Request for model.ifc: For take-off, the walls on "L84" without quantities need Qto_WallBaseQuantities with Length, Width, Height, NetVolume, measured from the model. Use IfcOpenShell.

First a look at what the model holds.

```python
import ifcopenshell
import ifcopenshell.util.element
import ifcopenshell.util.unit

model = ifcopenshell.open("model.ifc")
print(model.schema)
for unit_type in ("LENGTHUNIT", "AREAUNIT", "VOLUMEUNIT"):
    print(unit_type, ifcopenshell.util.unit.calculate_unit_scale(model, unit_type))
storey = next(s for s in model.by_type("IfcBuildingStorey") if s.Name == "L84")
walls = [e for e in ifcopenshell.util.element.get_decomposition(storey) if e.is_a("IfcWall")]
for e in sorted(walls, key=lambda e: e.id()):
    print(e.id(), e.is_a(), e.Name, list(ifcopenshell.util.element.get_psets(e, qtos_only=True)), sep=" | ")
```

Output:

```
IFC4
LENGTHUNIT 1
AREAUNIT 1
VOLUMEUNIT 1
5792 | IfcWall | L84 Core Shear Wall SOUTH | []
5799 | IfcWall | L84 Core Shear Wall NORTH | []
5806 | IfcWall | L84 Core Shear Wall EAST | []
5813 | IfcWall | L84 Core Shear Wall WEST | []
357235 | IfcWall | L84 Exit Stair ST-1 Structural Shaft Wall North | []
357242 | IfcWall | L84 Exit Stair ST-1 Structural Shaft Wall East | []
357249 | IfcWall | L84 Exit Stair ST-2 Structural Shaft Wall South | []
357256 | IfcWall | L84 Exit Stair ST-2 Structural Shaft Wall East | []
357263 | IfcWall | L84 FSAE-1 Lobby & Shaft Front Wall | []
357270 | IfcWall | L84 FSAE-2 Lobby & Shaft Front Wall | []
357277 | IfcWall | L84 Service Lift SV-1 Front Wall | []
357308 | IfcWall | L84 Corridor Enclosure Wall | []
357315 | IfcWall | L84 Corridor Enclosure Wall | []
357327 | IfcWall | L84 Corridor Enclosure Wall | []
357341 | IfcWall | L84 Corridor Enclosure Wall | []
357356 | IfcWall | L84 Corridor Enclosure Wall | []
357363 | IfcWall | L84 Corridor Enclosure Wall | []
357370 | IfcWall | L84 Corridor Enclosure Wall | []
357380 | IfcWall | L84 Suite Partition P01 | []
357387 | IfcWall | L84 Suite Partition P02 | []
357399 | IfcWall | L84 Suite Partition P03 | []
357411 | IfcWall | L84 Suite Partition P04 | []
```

```python
import ifcopenshell
import ifcopenshell.api.pset
import ifcopenshell.geom
import ifcopenshell.util.element
import ifcopenshell.util.shape
import ifcopenshell.util.unit

model = ifcopenshell.open("model.ifc")
unit_scale = ifcopenshell.util.unit.calculate_unit_scale(model)
volume_scale = ifcopenshell.util.unit.calculate_unit_scale(model, "VOLUMEUNIT")
settings = ifcopenshell.geom.settings()

storey = next(s for s in model.by_type("IfcBuildingStorey") if s.Name == "L84")
walls = [e for e in ifcopenshell.util.element.get_decomposition(storey) if e.is_a("IfcWall")]

for e in sorted(walls, key=lambda e: e.id()):
    if ifcopenshell.util.element.get_psets(e, qtos_only=True, should_inherit=False):
        continue
    # Geometry comes back in metres, in the element's own axes.
    shape = ifcopenshell.geom.create_shape(settings, e)
    values = {
        "Length": ifcopenshell.util.shape.get_x(shape.geometry) / unit_scale,
        "Width": ifcopenshell.util.shape.get_y(shape.geometry) / unit_scale,
        "Height": ifcopenshell.util.shape.get_z(shape.geometry) / unit_scale,
        "NetVolume": ifcopenshell.util.shape.get_volume(shape.geometry) / volume_scale,
    }
    qto = ifcopenshell.api.pset.add_qto(model, product=e, name="Qto_WallBaseQuantities")
    ifcopenshell.api.pset.edit_qto(model, qto=qto, properties=values)
    print(e.id(), {k: round(v, 3) for k, v in values.items()})

model.write("model_updated.ifc")
```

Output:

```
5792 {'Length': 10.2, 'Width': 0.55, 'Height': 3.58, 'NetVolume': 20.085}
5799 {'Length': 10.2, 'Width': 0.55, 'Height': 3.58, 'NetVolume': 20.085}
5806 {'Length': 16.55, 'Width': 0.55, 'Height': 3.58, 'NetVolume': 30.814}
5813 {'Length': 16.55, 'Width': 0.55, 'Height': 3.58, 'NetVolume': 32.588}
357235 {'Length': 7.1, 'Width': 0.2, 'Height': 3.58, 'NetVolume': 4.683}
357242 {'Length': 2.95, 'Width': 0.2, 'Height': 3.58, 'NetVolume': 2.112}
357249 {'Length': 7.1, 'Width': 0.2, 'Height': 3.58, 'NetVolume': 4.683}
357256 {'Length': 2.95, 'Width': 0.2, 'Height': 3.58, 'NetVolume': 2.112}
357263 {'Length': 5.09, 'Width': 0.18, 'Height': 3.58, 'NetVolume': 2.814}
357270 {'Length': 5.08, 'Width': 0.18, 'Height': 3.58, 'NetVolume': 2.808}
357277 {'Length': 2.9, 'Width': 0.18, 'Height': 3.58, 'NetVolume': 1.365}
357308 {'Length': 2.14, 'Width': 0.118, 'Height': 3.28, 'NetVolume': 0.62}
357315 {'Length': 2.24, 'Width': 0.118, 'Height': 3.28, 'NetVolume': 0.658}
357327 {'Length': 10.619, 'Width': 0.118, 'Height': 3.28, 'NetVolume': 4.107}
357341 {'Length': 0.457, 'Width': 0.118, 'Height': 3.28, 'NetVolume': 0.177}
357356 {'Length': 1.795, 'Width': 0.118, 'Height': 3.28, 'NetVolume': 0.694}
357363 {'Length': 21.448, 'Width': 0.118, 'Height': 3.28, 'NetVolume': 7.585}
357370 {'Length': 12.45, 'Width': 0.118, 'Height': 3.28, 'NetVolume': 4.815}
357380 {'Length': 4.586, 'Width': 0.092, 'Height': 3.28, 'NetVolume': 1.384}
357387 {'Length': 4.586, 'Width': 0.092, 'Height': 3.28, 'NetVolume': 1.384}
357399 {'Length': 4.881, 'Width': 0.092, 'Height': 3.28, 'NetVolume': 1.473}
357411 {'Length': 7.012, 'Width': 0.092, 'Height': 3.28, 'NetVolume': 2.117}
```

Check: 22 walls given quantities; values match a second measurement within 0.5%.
